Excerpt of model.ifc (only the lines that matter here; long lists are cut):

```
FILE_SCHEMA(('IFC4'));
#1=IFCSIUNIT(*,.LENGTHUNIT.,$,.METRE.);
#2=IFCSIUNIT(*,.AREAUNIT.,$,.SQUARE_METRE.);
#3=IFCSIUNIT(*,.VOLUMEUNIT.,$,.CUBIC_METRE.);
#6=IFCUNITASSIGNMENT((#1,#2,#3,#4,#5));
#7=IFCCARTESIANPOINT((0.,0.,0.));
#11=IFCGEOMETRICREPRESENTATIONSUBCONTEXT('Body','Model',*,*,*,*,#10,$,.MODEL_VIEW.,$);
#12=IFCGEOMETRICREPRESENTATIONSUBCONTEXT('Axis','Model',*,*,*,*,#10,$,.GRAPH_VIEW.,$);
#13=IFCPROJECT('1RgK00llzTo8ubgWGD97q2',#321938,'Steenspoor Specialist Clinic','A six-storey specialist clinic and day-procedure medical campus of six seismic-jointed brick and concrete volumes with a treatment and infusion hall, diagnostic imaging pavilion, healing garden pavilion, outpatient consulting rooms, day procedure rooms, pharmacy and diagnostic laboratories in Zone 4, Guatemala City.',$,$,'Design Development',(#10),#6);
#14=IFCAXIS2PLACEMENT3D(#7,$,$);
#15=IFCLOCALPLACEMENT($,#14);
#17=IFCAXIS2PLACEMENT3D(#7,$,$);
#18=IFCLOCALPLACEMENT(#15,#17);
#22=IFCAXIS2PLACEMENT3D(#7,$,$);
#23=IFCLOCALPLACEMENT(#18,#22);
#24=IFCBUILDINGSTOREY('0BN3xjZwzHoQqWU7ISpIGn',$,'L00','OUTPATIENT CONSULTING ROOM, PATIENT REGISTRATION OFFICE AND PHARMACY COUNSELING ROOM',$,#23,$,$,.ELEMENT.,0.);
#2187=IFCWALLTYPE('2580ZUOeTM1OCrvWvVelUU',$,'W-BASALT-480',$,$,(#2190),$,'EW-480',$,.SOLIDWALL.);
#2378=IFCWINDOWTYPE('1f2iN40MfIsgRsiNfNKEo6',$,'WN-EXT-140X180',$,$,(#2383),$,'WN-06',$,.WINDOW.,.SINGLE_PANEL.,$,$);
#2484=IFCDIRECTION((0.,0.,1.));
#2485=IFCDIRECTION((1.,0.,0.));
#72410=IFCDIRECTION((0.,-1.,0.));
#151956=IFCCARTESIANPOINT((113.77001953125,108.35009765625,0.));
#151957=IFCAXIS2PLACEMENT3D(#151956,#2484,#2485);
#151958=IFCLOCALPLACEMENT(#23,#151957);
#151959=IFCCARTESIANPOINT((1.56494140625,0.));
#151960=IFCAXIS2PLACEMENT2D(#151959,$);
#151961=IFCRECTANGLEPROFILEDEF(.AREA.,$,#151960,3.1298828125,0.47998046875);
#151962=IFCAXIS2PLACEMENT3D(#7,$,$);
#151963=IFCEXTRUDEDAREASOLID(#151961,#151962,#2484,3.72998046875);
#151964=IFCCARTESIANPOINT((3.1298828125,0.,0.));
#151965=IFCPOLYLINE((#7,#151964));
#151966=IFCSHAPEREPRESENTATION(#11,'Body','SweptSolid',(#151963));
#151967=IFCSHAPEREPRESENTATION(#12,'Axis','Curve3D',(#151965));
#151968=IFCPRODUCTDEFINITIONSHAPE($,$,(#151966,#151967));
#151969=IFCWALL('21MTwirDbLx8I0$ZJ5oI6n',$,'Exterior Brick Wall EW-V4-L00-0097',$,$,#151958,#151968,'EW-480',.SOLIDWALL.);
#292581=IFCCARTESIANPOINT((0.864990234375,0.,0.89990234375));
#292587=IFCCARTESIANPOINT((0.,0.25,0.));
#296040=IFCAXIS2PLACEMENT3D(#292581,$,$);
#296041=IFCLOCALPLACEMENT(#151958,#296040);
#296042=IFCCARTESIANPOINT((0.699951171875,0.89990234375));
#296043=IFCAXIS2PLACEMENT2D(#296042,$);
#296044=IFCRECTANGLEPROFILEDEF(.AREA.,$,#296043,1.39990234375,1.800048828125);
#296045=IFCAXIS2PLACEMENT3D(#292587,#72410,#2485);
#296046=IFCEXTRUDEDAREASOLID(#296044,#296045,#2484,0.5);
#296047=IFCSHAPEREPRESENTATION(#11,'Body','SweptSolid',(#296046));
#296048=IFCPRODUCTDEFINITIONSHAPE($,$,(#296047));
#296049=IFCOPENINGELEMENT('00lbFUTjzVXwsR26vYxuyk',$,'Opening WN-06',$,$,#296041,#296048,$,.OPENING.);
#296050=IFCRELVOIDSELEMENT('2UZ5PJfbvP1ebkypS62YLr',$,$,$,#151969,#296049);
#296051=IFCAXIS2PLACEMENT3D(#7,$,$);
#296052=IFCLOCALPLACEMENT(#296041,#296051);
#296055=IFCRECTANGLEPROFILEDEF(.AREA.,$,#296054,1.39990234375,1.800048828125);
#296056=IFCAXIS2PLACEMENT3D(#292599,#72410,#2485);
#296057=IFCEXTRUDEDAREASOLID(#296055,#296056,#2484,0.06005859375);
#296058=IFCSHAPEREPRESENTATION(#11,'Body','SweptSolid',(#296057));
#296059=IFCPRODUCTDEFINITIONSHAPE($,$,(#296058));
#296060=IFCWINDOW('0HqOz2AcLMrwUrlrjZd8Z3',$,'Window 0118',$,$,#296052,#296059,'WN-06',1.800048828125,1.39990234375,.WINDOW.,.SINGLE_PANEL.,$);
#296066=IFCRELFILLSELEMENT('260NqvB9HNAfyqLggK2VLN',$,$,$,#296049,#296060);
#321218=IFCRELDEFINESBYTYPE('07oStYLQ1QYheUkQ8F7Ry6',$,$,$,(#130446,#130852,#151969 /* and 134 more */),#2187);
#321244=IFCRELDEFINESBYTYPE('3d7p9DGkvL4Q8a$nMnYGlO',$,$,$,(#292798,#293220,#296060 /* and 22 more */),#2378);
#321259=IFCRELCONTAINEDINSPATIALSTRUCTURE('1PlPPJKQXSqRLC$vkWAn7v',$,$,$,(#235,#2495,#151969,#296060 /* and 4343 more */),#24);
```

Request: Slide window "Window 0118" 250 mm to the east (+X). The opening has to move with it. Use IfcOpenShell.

```python
import ifcopenshell
import ifcopenshell.api.geometry
import ifcopenshell.util.placement
import ifcopenshell.util.unit

model = ifcopenshell.open("model.ifc")
unit_scale = ifcopenshell.util.unit.calculate_unit_scale(model)

window = model.by_guid("0HqOz2AcLMrwUrlrjZd8Z3")
opening = window.FillsVoids[0].RelatingOpeningElement
wall = opening.VoidsElements[0].RelatingBuildingElement

wall_matrix = ifcopenshell.util.placement.get_local_placement(wall.ObjectPlacement)
shift = wall_matrix[:3, 0] * 0.25 / unit_scale
before = ifcopenshell.util.placement.get_local_placement(window.ObjectPlacement)[:3, 3].copy()

# The window is placed relative to its opening, so it follows when the opening moves.
matrix = ifcopenshell.util.placement.get_local_placement(opening.ObjectPlacement)
matrix[:3, 3] += shift
ifcopenshell.api.geometry.edit_object_placement(
    model, product=opening, matrix=matrix, is_si=False, should_transform_children=True
)

after = ifcopenshell.util.placement.get_local_placement(window.ObjectPlacement)[:3, 3]
print("window moved by", (after - before).round(3) + 0.0)

model.write("model_edited.ifc")
```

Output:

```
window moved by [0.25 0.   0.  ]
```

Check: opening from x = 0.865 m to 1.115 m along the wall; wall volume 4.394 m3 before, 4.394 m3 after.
